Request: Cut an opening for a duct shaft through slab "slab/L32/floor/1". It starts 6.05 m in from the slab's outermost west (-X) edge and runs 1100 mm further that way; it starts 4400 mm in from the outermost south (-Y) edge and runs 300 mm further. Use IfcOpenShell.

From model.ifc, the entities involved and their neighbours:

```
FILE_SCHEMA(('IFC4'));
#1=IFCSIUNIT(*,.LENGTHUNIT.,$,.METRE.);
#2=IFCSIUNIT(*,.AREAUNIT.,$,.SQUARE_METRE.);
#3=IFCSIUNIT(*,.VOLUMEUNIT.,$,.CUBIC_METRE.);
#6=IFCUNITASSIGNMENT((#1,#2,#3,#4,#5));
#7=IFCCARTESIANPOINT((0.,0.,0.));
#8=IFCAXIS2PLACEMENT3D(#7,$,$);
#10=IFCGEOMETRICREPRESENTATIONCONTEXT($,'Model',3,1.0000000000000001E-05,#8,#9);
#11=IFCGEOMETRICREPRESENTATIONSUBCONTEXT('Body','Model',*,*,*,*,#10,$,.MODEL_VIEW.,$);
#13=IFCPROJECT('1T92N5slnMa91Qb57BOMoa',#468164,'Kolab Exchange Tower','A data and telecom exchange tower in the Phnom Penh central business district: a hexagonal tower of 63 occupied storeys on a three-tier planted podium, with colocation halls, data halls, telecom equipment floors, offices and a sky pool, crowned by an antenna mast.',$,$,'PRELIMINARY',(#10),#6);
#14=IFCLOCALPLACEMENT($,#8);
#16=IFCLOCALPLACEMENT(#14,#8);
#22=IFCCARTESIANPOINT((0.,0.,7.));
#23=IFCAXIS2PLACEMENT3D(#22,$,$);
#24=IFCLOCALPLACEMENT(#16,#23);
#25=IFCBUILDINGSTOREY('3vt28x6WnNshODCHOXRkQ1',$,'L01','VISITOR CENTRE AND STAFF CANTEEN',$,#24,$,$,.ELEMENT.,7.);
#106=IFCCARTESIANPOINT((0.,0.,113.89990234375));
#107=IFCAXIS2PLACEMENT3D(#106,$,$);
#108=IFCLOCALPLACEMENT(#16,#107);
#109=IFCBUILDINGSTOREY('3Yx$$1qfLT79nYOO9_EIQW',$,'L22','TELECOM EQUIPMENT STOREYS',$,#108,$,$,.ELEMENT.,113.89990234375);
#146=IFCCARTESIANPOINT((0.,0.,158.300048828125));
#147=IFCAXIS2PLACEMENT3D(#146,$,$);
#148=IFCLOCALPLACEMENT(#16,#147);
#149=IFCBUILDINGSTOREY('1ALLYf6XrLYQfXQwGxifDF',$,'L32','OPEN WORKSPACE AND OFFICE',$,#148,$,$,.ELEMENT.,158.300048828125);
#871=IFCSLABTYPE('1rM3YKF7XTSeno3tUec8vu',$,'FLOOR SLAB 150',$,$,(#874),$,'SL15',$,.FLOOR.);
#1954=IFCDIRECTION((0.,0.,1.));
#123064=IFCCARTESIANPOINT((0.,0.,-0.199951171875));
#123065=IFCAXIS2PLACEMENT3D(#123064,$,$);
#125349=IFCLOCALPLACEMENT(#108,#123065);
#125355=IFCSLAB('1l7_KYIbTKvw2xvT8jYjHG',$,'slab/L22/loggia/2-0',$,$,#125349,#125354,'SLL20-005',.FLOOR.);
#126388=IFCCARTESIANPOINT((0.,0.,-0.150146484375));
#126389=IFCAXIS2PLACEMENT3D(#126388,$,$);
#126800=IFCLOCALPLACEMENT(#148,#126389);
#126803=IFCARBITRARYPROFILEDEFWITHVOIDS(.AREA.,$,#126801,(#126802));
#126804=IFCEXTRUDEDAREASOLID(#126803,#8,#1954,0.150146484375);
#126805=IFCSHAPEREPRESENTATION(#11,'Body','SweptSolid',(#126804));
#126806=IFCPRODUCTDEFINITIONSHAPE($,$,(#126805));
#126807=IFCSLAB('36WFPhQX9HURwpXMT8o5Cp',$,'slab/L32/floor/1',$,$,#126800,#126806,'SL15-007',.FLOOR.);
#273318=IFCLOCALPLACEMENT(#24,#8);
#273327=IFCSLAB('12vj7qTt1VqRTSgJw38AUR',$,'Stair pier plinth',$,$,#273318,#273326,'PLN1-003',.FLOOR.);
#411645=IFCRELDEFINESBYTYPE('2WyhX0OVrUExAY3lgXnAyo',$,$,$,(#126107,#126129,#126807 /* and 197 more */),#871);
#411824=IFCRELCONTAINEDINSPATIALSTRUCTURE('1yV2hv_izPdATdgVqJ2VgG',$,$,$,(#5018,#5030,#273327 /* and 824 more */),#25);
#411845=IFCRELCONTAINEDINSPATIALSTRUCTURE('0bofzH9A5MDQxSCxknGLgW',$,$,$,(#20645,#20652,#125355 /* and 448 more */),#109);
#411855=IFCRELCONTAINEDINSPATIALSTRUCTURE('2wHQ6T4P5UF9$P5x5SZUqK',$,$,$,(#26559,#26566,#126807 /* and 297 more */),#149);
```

```python
import numpy as np
import ifcopenshell
import ifcopenshell.api.feature
import ifcopenshell.api.geometry
import ifcopenshell.api.root
import ifcopenshell.geom
import ifcopenshell.util.placement
import ifcopenshell.util.representation
import ifcopenshell.util.shape
import ifcopenshell.util.unit

model = ifcopenshell.open("model.ifc")
unit_scale = ifcopenshell.util.unit.calculate_unit_scale(model)
settings = ifcopenshell.geom.settings()


def volume(element):
    """Net volume in cubic metres, openings subtracted."""
    shape = ifcopenshell.geom.create_shape(settings, element)
    return ifcopenshell.util.shape.get_volume(shape.geometry)


slab = model.by_id(126807)
before = volume(slab)

# Extent in the slab's own axes, in metres. The edges named are its -X and -Y sides.
slab_shape = ifcopenshell.geom.create_shape(settings, slab)
vertices = ifcopenshell.util.shape.get_vertices(slab_shape.geometry)
x_min, y_min, bottom = vertices.min(axis=0)
top = vertices[:, 2].max()

opening = ifcopenshell.api.root.create_entity(model, ifc_class="IfcOpeningElement", name="Duct shaft opening", predefined_type="OPENING")
context = ifcopenshell.util.representation.get_context(model, "Model", "Body", "MODEL_VIEW")
width, depth = 1.1, 0.3
outline = [(0.0, 0.0), (width, 0.0), (width, depth), (0.0, depth), (0.0, 0.0)]
# Overshoot both faces by 50 mm so the cut is clean.
shape = ifcopenshell.api.geometry.add_slab_representation(
    model, context=context, depth=top - bottom + 0.1, polyline=outline
)
ifcopenshell.api.geometry.assign_representation(model, product=opening, representation=shape)

matrix = ifcopenshell.util.placement.get_local_placement(slab.ObjectPlacement)
matrix[:, 3] = matrix @ np.append(np.array([x_min + 6.05, y_min + 4.4, bottom - 0.05]) / unit_scale, 1.0)
ifcopenshell.api.geometry.edit_object_placement(model, product=opening, matrix=matrix, is_si=False)
ifcopenshell.api.feature.add_feature(model, feature=opening, element=slab)

after = volume(slab)

print(f"slab volume {before:.3f} -> {after:.3f} m3")

model.write("model_edited.ifc")
```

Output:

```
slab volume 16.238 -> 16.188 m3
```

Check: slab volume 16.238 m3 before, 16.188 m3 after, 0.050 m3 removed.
